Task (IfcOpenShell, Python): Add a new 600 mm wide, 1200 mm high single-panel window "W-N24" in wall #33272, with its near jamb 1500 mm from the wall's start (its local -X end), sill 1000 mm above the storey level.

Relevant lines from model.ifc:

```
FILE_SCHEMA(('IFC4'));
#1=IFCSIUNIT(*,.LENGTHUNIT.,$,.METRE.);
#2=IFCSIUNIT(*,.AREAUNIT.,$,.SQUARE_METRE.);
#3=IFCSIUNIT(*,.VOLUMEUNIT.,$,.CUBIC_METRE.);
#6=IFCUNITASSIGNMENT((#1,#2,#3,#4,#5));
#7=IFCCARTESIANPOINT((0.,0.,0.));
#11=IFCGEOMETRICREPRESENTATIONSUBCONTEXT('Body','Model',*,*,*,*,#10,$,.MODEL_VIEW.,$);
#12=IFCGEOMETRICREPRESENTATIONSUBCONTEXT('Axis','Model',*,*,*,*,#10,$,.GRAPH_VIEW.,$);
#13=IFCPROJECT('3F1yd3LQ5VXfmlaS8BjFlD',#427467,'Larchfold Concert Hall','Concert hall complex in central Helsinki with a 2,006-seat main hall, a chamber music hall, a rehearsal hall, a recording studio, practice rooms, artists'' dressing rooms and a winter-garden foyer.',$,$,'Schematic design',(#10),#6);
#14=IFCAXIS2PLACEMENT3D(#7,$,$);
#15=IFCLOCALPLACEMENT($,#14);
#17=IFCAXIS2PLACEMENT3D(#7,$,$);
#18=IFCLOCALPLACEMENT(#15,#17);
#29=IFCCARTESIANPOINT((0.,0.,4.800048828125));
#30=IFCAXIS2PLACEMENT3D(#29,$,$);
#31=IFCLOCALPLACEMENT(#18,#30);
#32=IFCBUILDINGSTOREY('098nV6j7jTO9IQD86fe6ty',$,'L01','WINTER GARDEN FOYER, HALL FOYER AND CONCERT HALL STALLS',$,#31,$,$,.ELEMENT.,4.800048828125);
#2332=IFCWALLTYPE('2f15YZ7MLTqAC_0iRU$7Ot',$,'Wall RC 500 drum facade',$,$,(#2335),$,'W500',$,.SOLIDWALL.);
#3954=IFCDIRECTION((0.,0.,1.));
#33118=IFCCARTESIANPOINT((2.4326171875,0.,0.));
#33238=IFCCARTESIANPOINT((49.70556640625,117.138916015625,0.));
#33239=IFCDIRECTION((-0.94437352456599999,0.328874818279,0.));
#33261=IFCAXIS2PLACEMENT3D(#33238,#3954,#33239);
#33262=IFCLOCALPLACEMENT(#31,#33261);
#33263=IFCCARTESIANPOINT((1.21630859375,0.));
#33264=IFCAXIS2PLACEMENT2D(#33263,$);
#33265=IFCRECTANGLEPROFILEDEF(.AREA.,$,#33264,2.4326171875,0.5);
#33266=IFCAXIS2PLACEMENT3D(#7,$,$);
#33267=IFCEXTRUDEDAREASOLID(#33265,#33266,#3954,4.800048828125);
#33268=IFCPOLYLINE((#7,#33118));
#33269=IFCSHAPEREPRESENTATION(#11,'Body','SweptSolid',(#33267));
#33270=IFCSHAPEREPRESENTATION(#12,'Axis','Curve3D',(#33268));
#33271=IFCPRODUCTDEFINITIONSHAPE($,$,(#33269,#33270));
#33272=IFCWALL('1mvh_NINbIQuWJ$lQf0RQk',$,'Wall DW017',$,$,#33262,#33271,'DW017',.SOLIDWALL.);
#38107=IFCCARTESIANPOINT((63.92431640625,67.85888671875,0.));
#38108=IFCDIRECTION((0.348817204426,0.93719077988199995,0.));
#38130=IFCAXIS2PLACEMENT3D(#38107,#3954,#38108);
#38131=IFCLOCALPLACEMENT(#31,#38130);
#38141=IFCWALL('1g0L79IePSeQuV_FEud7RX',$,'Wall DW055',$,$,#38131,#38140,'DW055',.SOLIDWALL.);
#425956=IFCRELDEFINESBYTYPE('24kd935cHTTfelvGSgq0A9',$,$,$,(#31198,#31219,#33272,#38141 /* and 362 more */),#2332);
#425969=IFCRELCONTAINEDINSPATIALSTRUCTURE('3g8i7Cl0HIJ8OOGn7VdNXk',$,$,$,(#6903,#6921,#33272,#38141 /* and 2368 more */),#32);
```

```python
import numpy as np
import ifcopenshell
import ifcopenshell.api.feature
import ifcopenshell.api.geometry
import ifcopenshell.api.root
import ifcopenshell.api.spatial
import ifcopenshell.geom
import ifcopenshell.util.element
import ifcopenshell.util.placement
import ifcopenshell.util.representation
import ifcopenshell.util.shape
import ifcopenshell.util.unit

model = ifcopenshell.open("model.ifc")
unit_scale = ifcopenshell.util.unit.calculate_unit_scale(model)
settings = ifcopenshell.geom.settings()


def volume(element):
    """Net volume in cubic metres, openings subtracted."""
    shape = ifcopenshell.geom.create_shape(settings, element)
    return ifcopenshell.util.shape.get_volume(shape.geometry)


wall = model.by_guid("1mvh_NINbIQuWJ$lQf0RQk")
storey = ifcopenshell.util.element.get_container(wall, ifc_class="IfcBuildingStorey")
context = ifcopenshell.util.representation.get_context(model, "Model", "Body", "MODEL_VIEW")
before = volume(wall)

width, height, from_end, sill = 0.6, 1.2, 1.5, 1  # metres

# The wall runs along its own X axis, and the end named is its -X end.
wall_shape = ifcopenshell.geom.create_shape(settings, wall)
x, y, z = ifcopenshell.util.shape.get_vertices(wall_shape.geometry).T
start = x.min() + from_end
face, thickness = float(y.min()), float(y.max() - y.min())
wall_matrix = ifcopenshell.util.placement.get_local_placement(wall.ObjectPlacement)
level = ifcopenshell.util.placement.get_local_placement(storey.ObjectPlacement)[2, 3]


def in_wall(x, y):
    """Placement at x, y metres in the wall's axes, at sill height."""
    matrix = wall_matrix.copy()
    matrix[:, 3] = wall_matrix @ np.array([x / unit_scale, y / unit_scale, 0.0, 1.0])
    matrix[2, 3] = level + sill / unit_scale
    return matrix


# Opening: a box that overshoots both wall faces by 50 mm.
opening = ifcopenshell.api.root.create_entity(model, ifc_class="IfcOpeningElement", predefined_type="OPENING")
box = ifcopenshell.api.geometry.add_wall_representation(
    model, context=context, length=width, height=height, thickness=thickness + 0.1
)
ifcopenshell.api.geometry.assign_representation(model, product=opening, representation=box)
ifcopenshell.api.geometry.edit_object_placement(model, product=opening, matrix=in_wall(start, face - 0.05), is_si=False)
ifcopenshell.api.feature.add_feature(model, feature=opening, element=wall)

window = ifcopenshell.api.root.create_entity(model, ifc_class="IfcWindow", name="W-N24", predefined_type="WINDOW")
window.OverallWidth, window.OverallHeight = width / unit_scale, height / unit_scale
window.PartitioningType = "SINGLE_PANEL"
body = ifcopenshell.api.geometry.add_window_representation(
    model,
    context=context,
    overall_width=window.OverallWidth,
    overall_height=window.OverallHeight,
    partition_type="SINGLE_PANEL",
)
ifcopenshell.api.geometry.assign_representation(model, product=window, representation=body)
ifcopenshell.api.spatial.assign_container(model, products=[window], relating_structure=storey)
ifcopenshell.api.feature.add_filling(model, opening=opening, element=window)

# Centre the window in the wall's thickness.
ifcopenshell.api.geometry.edit_object_placement(model, product=window, matrix=in_wall(start, face), is_si=False)
window_shape = ifcopenshell.geom.create_shape(settings, window)
depth = ifcopenshell.util.shape.get_vertices(window_shape.geometry)[:, 1]
offset = face + thickness / 2 - (depth.min() + depth.max()) / 2
ifcopenshell.api.geometry.edit_object_placement(model, product=window, matrix=in_wall(start, offset), is_si=False)

after = volume(wall)

print(f"wall volume {before:.3f} -> {after:.3f} m3")

model.write("model_edited.ifc")
```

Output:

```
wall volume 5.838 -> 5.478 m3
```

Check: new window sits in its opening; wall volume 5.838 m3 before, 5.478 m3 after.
